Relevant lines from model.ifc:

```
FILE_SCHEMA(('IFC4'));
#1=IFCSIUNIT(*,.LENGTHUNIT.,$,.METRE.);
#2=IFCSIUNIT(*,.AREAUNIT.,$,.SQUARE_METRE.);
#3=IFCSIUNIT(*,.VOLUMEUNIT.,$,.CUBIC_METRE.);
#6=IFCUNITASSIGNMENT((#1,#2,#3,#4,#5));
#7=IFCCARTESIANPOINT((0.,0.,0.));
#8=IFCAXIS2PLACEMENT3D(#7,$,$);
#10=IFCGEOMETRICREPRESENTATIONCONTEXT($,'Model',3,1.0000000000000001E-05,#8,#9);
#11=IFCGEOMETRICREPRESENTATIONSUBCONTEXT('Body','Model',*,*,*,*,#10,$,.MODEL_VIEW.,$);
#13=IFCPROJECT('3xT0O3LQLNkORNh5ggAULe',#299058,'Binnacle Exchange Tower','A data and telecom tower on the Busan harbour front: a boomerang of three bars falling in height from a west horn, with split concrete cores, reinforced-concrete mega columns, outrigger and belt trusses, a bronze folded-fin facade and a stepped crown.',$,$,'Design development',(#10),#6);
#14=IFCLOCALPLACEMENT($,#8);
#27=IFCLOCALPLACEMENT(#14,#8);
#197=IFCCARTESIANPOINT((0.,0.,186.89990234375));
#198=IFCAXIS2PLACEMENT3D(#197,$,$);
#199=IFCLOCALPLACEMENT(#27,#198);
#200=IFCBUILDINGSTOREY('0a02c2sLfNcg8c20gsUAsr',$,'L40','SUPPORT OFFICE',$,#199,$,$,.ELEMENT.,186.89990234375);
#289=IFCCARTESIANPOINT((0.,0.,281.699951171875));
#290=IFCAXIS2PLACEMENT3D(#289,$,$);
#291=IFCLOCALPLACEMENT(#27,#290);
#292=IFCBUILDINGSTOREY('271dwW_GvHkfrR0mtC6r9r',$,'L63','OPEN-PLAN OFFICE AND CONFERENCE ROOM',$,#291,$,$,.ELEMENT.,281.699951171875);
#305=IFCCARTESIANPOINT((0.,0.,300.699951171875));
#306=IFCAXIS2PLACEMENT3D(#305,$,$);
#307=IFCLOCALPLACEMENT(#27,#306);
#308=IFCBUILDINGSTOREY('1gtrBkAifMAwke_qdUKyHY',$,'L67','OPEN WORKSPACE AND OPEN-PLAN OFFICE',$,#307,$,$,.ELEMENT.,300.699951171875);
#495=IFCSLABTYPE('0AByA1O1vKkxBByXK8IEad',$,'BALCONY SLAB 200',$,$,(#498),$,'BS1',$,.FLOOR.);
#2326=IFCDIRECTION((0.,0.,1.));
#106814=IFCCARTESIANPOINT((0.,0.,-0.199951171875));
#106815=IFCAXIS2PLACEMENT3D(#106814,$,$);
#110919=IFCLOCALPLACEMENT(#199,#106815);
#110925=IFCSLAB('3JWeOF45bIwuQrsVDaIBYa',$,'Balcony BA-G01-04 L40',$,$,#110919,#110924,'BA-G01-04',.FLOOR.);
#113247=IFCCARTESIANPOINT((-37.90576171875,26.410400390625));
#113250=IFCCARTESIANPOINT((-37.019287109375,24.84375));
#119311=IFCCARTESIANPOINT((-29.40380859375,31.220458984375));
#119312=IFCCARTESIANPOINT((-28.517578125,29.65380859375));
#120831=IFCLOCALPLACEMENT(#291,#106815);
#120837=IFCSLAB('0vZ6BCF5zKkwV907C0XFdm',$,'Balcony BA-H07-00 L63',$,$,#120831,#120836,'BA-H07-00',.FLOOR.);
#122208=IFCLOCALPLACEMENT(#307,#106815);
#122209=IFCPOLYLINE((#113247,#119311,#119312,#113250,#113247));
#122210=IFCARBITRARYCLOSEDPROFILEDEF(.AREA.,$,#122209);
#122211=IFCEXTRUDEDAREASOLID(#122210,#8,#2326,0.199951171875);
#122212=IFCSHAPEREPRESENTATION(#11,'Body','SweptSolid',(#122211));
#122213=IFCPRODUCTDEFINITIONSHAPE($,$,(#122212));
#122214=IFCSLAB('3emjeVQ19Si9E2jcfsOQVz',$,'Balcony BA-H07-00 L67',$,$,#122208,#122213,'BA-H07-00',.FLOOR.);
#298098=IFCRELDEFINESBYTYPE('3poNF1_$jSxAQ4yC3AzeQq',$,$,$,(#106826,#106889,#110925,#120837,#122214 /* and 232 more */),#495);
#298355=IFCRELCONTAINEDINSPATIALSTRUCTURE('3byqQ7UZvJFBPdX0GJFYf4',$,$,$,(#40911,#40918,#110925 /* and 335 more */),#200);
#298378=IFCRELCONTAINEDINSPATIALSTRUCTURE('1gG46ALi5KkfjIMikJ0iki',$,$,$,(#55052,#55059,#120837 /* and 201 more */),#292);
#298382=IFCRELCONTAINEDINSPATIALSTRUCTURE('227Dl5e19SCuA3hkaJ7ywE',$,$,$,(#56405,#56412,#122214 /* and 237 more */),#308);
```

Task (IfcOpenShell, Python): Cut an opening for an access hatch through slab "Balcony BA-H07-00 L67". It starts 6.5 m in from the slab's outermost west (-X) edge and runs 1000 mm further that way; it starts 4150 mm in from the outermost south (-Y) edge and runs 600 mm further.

```python
import numpy as np
import ifcopenshell
import ifcopenshell.api.feature
import ifcopenshell.api.geometry
import ifcopenshell.api.root
import ifcopenshell.geom
import ifcopenshell.util.placement
import ifcopenshell.util.representation
import ifcopenshell.util.shape
import ifcopenshell.util.unit

model = ifcopenshell.open("model.ifc")
unit_scale = ifcopenshell.util.unit.calculate_unit_scale(model)
settings = ifcopenshell.geom.settings()


def volume(element):
    """Net volume in cubic metres, openings subtracted."""
    shape = ifcopenshell.geom.create_shape(settings, element)
    return ifcopenshell.util.shape.get_volume(shape.geometry)


slab = model.by_guid("3emjeVQ19Si9E2jcfsOQVz")
before = volume(slab)

# Extent in the slab's own axes, in metres. The edges named are its -X and -Y sides.
slab_shape = ifcopenshell.geom.create_shape(settings, slab)
vertices = ifcopenshell.util.shape.get_vertices(slab_shape.geometry)
x_min, y_min, bottom = vertices.min(axis=0)
top = vertices[:, 2].max()

opening = ifcopenshell.api.root.create_entity(model, ifc_class="IfcOpeningElement", name="Access hatch opening", predefined_type="OPENING")
context = ifcopenshell.util.representation.get_context(model, "Model", "Body", "MODEL_VIEW")
width, depth = 1, 0.6
outline = [(0.0, 0.0), (width, 0.0), (width, depth), (0.0, depth), (0.0, 0.0)]
# Overshoot both faces by 50 mm so the cut is clean.
shape = ifcopenshell.api.geometry.add_slab_representation(
    model, context=context, depth=top - bottom + 0.1, polyline=outline
)
ifcopenshell.api.geometry.assign_representation(model, product=opening, representation=shape)

matrix = ifcopenshell.util.placement.get_local_placement(slab.ObjectPlacement)
matrix[:, 3] = matrix @ np.append(np.array([x_min + 6.5, y_min + 4.15, bottom - 0.05]) / unit_scale, 1.0)
ifcopenshell.api.geometry.edit_object_placement(model, product=opening, matrix=matrix, is_si=False)
ifcopenshell.api.feature.add_feature(model, feature=opening, element=slab)

after = volume(slab)

print(f"slab volume {before:.3f} -> {after:.3f} m3")

model.write("model_rev.ifc")
```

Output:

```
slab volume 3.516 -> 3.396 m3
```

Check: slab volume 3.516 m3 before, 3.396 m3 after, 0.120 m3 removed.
